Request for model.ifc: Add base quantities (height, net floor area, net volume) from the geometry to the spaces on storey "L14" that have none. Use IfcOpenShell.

First a look at what the model holds.

```python
import ifcopenshell
import ifcopenshell.util.element
import ifcopenshell.util.unit

model = ifcopenshell.open("model.ifc")
print(model.schema)
for unit_type in ("LENGTHUNIT", "AREAUNIT", "VOLUMEUNIT"):
    print(unit_type, ifcopenshell.util.unit.calculate_unit_scale(model, unit_type))
storey = next(s for s in model.by_type("IfcBuildingStorey") if s.Name == "L14")
spaces = [e for e in ifcopenshell.util.element.get_decomposition(storey) if e.is_a("IfcSpace")]
for e in sorted(spaces, key=lambda e: e.id()):
    print(e.id(), e.is_a(), e.Name, list(ifcopenshell.util.element.get_psets(e, qtos_only=True)), sep=" | ")
```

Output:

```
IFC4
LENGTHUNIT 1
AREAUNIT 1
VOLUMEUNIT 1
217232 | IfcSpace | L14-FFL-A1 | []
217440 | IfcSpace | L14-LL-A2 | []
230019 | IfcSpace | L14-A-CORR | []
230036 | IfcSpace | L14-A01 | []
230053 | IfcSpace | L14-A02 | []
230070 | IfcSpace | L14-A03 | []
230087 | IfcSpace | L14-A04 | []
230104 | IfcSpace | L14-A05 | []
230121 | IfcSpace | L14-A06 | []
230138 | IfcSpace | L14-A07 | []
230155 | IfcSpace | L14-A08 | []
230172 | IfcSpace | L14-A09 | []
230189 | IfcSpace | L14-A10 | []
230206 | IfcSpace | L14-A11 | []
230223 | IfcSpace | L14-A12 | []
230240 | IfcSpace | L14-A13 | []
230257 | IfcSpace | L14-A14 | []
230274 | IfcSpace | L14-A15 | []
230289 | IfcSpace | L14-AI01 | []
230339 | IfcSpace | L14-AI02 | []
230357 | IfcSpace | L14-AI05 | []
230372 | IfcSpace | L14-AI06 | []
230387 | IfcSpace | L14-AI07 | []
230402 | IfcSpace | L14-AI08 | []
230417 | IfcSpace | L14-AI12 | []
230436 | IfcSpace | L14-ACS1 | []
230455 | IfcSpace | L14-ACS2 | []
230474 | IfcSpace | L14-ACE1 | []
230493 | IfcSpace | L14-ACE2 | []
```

```python
import ifcopenshell
import ifcopenshell.api.pset
import ifcopenshell.geom
import ifcopenshell.util.element
import ifcopenshell.util.shape
import ifcopenshell.util.unit

model = ifcopenshell.open("model.ifc")
unit_scale = ifcopenshell.util.unit.calculate_unit_scale(model)
area_scale = ifcopenshell.util.unit.calculate_unit_scale(model, "AREAUNIT")
volume_scale = ifcopenshell.util.unit.calculate_unit_scale(model, "VOLUMEUNIT")
settings = ifcopenshell.geom.settings()

storey = next(s for s in model.by_type("IfcBuildingStorey") if s.Name == "L14")
spaces = [e for e in ifcopenshell.util.element.get_decomposition(storey) if e.is_a("IfcSpace")]

for e in sorted(spaces, key=lambda e: e.id()):
    if ifcopenshell.util.element.get_psets(e, qtos_only=True, should_inherit=False):
        continue
    # Geometry comes back in metres, in the element's own axes.
    shape = ifcopenshell.geom.create_shape(settings, e)
    values = {
        "Height": ifcopenshell.util.shape.get_z(shape.geometry) / unit_scale,
        "NetFloorArea": ifcopenshell.util.shape.get_footprint_area(shape.geometry) / area_scale,
        "NetVolume": ifcopenshell.util.shape.get_volume(shape.geometry) / volume_scale,
    }
    qto = ifcopenshell.api.pset.add_qto(model, product=e, name="Qto_SpaceBaseQuantities")
    ifcopenshell.api.pset.edit_qto(model, qto=qto, properties=values)
    print(e.id(), {k: round(v, 3) for k, v in values.items()})

model.write("model_edited.ifc")
```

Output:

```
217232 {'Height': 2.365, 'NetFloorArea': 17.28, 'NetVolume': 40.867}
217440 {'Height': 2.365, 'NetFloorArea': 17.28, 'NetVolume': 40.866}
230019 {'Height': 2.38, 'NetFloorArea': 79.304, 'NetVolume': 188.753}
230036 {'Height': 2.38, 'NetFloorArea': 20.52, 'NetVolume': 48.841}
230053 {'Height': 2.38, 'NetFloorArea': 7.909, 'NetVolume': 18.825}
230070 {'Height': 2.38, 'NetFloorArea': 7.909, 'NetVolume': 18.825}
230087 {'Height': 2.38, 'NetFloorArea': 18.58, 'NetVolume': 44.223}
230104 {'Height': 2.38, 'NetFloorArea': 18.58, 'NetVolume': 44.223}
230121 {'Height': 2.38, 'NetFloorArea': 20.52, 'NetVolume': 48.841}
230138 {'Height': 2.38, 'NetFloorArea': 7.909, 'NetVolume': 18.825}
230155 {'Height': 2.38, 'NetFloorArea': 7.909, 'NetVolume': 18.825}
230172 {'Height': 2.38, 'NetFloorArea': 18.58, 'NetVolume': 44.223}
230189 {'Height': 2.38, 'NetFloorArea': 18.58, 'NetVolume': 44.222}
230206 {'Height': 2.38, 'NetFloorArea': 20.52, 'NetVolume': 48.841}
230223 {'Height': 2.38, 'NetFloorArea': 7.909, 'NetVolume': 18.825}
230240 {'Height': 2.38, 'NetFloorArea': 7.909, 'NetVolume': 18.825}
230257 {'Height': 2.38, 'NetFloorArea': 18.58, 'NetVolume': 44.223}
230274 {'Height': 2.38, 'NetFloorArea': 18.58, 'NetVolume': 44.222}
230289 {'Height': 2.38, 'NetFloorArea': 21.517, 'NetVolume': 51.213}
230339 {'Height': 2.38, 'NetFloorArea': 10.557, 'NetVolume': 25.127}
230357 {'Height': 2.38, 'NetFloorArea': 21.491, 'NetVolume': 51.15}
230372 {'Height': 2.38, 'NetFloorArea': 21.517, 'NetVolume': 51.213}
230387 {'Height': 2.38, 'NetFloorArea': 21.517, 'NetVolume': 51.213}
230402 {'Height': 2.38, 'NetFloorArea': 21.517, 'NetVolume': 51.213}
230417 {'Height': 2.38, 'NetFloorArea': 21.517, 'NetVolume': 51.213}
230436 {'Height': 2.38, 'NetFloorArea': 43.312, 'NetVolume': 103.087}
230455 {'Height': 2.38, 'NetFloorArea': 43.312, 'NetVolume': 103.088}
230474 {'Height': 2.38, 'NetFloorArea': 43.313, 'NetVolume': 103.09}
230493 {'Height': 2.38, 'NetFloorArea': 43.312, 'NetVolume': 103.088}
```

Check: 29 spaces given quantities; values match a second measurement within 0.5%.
